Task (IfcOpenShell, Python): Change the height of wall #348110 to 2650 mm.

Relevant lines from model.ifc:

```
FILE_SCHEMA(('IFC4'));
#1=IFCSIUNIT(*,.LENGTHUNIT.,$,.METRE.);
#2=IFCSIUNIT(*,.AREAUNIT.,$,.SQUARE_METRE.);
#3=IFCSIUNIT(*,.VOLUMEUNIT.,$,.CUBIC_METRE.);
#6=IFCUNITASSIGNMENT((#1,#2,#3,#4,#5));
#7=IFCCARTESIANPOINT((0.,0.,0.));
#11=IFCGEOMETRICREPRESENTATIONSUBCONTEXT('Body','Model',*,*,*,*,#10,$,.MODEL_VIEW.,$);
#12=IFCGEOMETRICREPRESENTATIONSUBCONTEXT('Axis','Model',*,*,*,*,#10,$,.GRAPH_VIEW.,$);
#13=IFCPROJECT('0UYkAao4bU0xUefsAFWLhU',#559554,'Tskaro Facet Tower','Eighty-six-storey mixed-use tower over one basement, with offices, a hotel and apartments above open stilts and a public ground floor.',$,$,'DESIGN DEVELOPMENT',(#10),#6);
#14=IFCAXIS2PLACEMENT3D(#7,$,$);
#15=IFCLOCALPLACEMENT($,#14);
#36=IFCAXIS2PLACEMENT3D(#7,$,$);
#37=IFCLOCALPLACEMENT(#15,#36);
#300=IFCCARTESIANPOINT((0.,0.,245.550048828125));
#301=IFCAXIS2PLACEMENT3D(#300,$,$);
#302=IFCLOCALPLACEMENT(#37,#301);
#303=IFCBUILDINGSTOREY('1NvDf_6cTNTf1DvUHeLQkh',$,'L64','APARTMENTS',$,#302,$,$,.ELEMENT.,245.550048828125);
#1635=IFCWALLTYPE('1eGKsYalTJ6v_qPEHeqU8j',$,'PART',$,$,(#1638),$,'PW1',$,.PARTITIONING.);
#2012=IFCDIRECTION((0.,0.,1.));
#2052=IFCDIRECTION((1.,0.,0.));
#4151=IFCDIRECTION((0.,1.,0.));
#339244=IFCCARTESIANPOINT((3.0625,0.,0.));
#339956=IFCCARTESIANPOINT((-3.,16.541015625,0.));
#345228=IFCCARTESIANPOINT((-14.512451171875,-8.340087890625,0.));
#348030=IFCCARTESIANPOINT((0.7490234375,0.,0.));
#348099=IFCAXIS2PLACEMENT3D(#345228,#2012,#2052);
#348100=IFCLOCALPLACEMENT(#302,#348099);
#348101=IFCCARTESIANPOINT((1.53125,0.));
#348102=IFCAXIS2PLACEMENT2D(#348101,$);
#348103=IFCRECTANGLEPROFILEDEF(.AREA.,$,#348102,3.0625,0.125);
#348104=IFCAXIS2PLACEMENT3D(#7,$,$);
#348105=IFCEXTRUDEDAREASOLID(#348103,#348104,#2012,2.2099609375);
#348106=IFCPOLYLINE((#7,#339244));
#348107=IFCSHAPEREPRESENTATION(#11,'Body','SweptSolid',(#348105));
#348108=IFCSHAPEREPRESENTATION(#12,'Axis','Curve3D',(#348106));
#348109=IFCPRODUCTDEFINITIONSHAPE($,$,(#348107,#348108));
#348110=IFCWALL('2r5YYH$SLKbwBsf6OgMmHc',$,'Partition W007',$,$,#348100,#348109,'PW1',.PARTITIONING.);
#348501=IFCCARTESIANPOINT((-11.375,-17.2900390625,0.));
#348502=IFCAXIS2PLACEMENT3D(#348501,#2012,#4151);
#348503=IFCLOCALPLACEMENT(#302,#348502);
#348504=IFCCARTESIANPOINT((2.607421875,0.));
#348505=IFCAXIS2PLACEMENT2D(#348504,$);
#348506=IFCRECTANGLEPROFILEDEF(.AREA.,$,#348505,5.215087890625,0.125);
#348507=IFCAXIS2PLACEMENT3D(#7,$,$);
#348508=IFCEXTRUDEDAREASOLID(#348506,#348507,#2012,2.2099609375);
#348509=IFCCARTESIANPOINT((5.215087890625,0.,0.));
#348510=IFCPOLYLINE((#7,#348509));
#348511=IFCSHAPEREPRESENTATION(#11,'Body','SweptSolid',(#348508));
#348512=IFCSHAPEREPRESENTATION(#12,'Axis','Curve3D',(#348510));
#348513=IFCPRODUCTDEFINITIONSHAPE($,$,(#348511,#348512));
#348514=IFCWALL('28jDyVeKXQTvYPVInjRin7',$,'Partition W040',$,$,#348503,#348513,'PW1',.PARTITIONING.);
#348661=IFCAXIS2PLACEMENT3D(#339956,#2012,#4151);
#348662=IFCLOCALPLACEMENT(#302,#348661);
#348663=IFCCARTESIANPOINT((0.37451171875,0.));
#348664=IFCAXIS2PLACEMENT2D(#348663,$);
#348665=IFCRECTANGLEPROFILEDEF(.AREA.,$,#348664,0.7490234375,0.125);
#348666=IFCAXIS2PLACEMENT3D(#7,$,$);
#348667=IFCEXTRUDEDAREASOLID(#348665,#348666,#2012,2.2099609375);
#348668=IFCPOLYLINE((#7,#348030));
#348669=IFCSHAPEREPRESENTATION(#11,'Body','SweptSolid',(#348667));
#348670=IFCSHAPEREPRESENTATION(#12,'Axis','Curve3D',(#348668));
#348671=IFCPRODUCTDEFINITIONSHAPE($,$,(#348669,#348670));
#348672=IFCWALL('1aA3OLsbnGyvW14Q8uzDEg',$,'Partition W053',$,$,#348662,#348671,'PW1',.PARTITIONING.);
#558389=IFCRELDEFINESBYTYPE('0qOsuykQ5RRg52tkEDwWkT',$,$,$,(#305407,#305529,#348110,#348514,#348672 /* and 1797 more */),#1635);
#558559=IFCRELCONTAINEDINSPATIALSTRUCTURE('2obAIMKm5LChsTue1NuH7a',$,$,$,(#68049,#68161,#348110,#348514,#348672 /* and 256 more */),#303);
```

```python
import ifcopenshell
import ifcopenshell.geom
import ifcopenshell.util.representation
import ifcopenshell.util.shape
import ifcopenshell.util.unit

model = ifcopenshell.open("model.ifc")
unit_scale = ifcopenshell.util.unit.calculate_unit_scale(model)
settings = ifcopenshell.geom.settings()


def volume(element):
    """Net volume in cubic metres, openings subtracted."""
    shape = ifcopenshell.geom.create_shape(settings, element)
    return ifcopenshell.util.shape.get_volume(shape.geometry)


wall = model.by_id(348110)
before = volume(wall)

body = ifcopenshell.util.representation.get_representation(wall, "Model", "Body")
solid = body.Items[0]
old_height = solid.Depth
solid.Depth = 2.65 / unit_scale
after = volume(wall)

print(f"height {old_height:g} -> {solid.Depth:g}, volume {before:.3f} -> {after:.3f} m3")

model.write("model_rev.ifc")
```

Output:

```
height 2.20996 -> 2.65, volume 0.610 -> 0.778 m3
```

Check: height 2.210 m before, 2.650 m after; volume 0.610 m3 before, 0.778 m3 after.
